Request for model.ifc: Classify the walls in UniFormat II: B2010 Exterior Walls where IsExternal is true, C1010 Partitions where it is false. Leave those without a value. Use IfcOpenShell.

First a look at what the model holds.

```python
import ifcopenshell
import ifcopenshell.util.element

model = ifcopenshell.open("model.ifc")
print(model.schema)
print("classifications:", [c.Name for c in model.by_type("IfcClassification")])
values = [ifcopenshell.util.element.get_pset(e, "Pset_WallCommon", "IsExternal") for e in model.by_type("IfcWall")]
for value in (True, False, None):
    print("IsExternal", value, values.count(value))
```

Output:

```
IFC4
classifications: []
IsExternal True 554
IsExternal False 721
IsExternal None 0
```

```python
import ifcopenshell
import ifcopenshell.api.classification
import ifcopenshell.util.element

model = ifcopenshell.open("model.ifc")

system = ifcopenshell.api.classification.add_classification(model, classification="UniFormat II")

walls = model.by_type("IfcWall")
external = {e: ifcopenshell.util.element.get_pset(e, "Pset_WallCommon", "IsExternal") for e in walls}
for flag, code, name in ((True, "B2010", "Exterior Walls"), (False, "C1010", "Partitions")):
    products = [e for e in walls if external[e] is flag]
    ifcopenshell.api.classification.add_reference(
        model, products=products, classification=system, identification=code, name=name
    )
    print(code, len(products))

model.write("model_updated.ifc")
```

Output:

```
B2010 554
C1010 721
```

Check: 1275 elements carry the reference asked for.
